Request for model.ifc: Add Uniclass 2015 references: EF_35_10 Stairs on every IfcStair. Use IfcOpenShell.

First a look at what the model holds.

```python
import ifcopenshell

model = ifcopenshell.open("model.ifc")
print(model.schema)
print("classifications:", [c.Name for c in model.by_type("IfcClassification")])
for ifc_class in ("IfcDoor", "IfcRoof", "IfcStair", "IfcWall", "IfcWindow"):
    print(ifc_class, len(model.by_type(ifc_class)))
```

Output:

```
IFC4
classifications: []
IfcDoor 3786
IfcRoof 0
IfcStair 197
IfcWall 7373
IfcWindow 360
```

```python
import ifcopenshell
import ifcopenshell.api.classification

model = ifcopenshell.open("model.ifc")

system = ifcopenshell.api.classification.add_classification(model, classification="Uniclass 2015")

codes = {
    "IfcStair": ("EF_35_10", "Stairs"),
}
for ifc_class, (code, name) in codes.items():
    products = model.by_type(ifc_class)
    ifcopenshell.api.classification.add_reference(
        model, products=products, classification=system, identification=code, name=name
    )
    print(code, len(products))

model.write("model_edited.ifc")
```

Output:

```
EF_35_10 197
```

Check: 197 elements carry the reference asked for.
